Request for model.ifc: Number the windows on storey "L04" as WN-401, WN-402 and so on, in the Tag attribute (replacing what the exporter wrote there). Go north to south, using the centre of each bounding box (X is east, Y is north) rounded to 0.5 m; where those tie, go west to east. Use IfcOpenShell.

First a look at what the model holds.

```python
import ifcopenshell
import ifcopenshell.util.element
import ifcopenshell.util.placement

model = ifcopenshell.open("model.ifc")
print(model.schema)
storey = next(s for s in model.by_type("IfcBuildingStorey") if s.Name == "L04")
windows = [e for e in ifcopenshell.util.element.get_decomposition(storey) if e.is_a("IfcWindow")]
for e in sorted(windows, key=lambda e: e.id()):
    origin = ifcopenshell.util.placement.get_local_placement(e.ObjectPlacement)[:3, 3]
    print(e.id(), e.Tag, e.Name, origin.round(2) + 0.0, sep=" | ")
```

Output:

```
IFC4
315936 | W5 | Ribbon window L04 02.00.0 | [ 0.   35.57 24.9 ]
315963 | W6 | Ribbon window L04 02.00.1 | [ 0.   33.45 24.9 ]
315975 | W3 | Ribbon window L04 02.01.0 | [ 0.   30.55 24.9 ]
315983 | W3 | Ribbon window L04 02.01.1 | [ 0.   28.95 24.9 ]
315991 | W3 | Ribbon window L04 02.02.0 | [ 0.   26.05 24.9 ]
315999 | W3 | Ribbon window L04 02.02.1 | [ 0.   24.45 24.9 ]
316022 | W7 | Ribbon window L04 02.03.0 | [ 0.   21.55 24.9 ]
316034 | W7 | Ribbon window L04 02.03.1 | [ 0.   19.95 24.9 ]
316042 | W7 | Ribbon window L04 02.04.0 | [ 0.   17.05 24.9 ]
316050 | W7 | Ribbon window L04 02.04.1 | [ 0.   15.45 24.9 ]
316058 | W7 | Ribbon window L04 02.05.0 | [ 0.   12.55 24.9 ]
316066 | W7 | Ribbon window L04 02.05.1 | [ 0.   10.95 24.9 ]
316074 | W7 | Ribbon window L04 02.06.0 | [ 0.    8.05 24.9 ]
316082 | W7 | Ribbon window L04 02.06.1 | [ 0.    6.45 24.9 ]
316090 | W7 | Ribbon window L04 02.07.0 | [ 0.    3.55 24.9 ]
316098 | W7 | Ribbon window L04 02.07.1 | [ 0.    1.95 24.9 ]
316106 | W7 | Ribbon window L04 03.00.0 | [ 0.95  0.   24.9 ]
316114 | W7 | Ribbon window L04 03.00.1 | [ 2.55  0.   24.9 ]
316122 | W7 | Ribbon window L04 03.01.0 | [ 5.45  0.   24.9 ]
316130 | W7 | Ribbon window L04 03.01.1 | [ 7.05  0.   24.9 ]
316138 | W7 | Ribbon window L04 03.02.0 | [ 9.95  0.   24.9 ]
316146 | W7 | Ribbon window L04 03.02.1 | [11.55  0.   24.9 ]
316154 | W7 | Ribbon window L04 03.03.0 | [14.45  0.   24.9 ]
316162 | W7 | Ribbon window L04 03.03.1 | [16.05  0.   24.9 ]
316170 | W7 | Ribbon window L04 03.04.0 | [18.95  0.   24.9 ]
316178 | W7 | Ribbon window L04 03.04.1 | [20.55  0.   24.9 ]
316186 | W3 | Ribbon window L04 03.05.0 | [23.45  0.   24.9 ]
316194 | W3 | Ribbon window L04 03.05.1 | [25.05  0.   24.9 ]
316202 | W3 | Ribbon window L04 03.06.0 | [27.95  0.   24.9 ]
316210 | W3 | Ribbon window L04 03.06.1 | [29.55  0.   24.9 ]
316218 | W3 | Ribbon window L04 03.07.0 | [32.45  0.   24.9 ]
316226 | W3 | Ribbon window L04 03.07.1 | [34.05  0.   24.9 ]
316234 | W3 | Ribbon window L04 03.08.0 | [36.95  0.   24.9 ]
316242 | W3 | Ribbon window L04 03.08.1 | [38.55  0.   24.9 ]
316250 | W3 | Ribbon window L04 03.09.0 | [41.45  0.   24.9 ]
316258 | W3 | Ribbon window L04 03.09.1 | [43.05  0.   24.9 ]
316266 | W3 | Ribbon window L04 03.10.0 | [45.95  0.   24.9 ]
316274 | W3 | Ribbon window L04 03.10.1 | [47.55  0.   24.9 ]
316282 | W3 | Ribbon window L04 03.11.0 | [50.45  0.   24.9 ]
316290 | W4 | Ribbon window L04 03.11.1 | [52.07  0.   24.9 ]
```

```python
import ifcopenshell
import ifcopenshell.geom
import ifcopenshell.util.element
import ifcopenshell.util.shape

model = ifcopenshell.open("model.ifc")
settings = ifcopenshell.geom.settings()
settings.set("use-world-coords", True)


def centre(element):
    shape = ifcopenshell.geom.create_shape(settings, element)
    return ifcopenshell.util.shape.get_bbox_centroid(shape.geometry)


storey = next(s for s in model.by_type("IfcBuildingStorey") if s.Name == "L04")
windows = [e for e in ifcopenshell.util.element.get_decomposition(storey) if e.is_a("IfcWindow")]

# Insertion points can sit at a corner or the storey origin, so sort by the geometry (in metres).
centres = {e: centre(e) for e in windows}
windows.sort(key=lambda e: (-round(centres[e][1] / 0.5), centres[e][0]))

for i, e in enumerate(windows, start=1):
    number = f"WN-4{i:02d}"
    e.Tag = number
    print(e.id(), number)

model.write("model_updated.ifc")
```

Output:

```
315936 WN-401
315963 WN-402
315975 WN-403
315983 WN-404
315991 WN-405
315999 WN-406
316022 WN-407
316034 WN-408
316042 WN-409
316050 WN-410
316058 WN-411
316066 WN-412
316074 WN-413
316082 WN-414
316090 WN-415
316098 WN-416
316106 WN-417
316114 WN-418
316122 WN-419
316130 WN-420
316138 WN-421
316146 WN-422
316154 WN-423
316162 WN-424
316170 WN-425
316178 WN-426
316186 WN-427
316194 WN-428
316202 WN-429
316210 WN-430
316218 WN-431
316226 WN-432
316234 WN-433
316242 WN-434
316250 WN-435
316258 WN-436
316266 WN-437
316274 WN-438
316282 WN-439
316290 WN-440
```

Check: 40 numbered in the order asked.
